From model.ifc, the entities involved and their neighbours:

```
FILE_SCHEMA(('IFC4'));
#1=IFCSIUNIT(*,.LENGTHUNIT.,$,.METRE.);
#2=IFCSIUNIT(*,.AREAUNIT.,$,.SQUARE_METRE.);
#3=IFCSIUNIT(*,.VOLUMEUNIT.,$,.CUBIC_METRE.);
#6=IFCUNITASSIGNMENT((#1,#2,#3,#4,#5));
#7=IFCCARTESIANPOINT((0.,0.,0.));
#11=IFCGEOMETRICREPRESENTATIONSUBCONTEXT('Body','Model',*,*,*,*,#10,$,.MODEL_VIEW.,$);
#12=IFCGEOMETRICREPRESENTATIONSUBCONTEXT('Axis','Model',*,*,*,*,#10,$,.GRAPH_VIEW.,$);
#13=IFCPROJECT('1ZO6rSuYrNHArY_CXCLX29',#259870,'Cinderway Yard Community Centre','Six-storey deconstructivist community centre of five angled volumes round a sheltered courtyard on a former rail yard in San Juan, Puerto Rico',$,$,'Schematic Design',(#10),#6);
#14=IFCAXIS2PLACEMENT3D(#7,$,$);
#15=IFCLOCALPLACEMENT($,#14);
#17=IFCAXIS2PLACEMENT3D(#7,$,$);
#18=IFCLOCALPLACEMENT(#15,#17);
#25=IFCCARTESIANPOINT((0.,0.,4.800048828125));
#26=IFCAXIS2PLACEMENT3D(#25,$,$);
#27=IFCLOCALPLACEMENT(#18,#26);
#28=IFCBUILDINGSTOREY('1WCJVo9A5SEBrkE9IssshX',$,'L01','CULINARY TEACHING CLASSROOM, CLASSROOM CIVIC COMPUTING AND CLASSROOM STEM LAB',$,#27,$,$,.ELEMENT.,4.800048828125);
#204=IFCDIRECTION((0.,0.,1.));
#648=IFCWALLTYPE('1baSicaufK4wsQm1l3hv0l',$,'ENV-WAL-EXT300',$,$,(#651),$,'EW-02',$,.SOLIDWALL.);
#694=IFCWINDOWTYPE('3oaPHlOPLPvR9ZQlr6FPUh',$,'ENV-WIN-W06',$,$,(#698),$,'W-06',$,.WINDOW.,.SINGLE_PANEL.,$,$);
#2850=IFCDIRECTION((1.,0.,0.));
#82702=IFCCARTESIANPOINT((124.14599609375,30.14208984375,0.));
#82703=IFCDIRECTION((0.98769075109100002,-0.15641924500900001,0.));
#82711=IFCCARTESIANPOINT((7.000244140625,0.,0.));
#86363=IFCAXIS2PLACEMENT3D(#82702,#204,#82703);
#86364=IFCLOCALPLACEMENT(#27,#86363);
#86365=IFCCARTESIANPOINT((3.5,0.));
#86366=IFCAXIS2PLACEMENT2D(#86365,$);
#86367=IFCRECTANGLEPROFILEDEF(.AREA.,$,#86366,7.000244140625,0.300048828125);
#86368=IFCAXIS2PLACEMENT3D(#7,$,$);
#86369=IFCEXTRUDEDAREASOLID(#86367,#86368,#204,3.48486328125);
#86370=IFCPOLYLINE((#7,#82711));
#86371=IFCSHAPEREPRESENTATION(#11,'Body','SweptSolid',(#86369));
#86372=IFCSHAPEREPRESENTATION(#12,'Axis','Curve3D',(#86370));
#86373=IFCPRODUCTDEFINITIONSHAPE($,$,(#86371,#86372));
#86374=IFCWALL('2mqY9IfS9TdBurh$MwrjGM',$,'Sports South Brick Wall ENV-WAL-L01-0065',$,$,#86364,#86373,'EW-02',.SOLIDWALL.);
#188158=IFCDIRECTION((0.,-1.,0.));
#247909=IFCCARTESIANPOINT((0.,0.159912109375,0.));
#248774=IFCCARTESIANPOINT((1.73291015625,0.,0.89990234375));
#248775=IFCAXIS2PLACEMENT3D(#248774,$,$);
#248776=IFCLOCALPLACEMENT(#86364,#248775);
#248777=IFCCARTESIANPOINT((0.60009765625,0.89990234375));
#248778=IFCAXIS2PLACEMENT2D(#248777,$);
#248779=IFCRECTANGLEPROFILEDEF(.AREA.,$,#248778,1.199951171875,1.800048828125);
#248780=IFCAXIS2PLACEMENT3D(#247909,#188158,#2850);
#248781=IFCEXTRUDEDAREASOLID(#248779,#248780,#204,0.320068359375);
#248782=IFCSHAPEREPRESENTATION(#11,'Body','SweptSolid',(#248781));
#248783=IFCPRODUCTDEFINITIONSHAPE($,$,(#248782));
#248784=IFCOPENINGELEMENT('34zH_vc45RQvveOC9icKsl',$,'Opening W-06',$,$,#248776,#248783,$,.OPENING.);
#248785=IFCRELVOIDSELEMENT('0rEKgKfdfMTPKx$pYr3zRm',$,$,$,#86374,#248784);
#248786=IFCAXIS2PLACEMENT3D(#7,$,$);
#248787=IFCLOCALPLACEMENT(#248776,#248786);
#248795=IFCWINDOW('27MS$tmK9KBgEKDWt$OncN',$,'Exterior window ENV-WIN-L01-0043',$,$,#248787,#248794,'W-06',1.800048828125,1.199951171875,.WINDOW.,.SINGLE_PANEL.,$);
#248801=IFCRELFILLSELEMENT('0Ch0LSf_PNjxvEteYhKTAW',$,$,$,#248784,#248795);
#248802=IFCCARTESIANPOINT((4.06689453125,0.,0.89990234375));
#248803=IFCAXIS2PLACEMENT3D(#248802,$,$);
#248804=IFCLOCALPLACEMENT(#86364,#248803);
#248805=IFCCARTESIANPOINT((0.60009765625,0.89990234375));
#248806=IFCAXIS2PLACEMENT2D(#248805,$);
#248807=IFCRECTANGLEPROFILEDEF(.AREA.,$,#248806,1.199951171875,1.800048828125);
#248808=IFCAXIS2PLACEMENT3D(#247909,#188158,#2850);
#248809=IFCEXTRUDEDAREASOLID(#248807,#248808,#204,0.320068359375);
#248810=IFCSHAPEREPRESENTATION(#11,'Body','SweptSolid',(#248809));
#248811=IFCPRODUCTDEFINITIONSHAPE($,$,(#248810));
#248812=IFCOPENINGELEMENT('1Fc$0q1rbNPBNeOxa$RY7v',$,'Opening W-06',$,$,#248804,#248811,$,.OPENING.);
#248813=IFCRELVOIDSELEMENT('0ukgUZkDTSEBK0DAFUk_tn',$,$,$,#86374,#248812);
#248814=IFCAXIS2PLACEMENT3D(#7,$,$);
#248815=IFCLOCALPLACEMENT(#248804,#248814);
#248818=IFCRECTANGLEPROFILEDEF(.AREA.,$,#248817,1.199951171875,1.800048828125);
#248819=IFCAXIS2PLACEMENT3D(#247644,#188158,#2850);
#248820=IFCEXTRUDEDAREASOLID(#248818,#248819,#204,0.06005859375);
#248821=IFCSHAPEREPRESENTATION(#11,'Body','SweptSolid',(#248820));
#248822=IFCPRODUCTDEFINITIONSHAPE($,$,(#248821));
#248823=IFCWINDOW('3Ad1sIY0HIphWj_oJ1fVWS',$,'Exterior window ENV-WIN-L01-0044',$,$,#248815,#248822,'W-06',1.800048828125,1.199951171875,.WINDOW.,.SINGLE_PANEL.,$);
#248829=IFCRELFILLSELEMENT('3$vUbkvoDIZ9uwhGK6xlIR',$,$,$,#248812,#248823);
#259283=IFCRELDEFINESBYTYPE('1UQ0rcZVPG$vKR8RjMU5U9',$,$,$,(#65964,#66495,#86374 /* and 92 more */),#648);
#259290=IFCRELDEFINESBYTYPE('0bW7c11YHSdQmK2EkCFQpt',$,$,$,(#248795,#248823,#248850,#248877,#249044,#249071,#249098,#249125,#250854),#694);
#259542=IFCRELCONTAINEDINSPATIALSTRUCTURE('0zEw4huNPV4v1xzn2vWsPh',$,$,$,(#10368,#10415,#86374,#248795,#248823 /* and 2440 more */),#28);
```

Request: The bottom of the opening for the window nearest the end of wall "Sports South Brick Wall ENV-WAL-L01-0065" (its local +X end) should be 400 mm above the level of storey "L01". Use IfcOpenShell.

```python
import numpy as np
import ifcopenshell
import ifcopenshell.api.geometry
import ifcopenshell.geom
import ifcopenshell.util.element
import ifcopenshell.util.placement
import ifcopenshell.util.shape
import ifcopenshell.util.unit

model = ifcopenshell.open("model.ifc")
unit_scale = ifcopenshell.util.unit.calculate_unit_scale(model)

window = model.by_id(248823)
opening = window.FillsVoids[0].RelatingOpeningElement
storey = ifcopenshell.util.element.get_container(window, ifc_class="IfcBuildingStorey")
level = ifcopenshell.util.placement.get_local_placement(storey.ObjectPlacement)[2, 3]

# The opening's origin need not be at the sill, so measure its lowest point.
shape = ifcopenshell.geom.create_shape(ifcopenshell.geom.settings(), opening)
bottom = ifcopenshell.util.shape.get_shape_bottom_elevation(shape, shape.geometry) / unit_scale
dz = level + 0.4 / unit_scale - bottom

shift = np.array([0.0, 0.0, dz])
# The window is placed relative to its opening, so it follows when the opening moves.
matrix = ifcopenshell.util.placement.get_local_placement(opening.ObjectPlacement)
matrix[:3, 3] += shift
ifcopenshell.api.geometry.edit_object_placement(
    model, product=opening, matrix=matrix, is_si=False, should_transform_children=True
)

print(f"moved by {dz * unit_scale:+.3f} m")

model.write("model_v2.ifc")
```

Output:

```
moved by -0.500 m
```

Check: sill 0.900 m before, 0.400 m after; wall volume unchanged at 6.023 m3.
